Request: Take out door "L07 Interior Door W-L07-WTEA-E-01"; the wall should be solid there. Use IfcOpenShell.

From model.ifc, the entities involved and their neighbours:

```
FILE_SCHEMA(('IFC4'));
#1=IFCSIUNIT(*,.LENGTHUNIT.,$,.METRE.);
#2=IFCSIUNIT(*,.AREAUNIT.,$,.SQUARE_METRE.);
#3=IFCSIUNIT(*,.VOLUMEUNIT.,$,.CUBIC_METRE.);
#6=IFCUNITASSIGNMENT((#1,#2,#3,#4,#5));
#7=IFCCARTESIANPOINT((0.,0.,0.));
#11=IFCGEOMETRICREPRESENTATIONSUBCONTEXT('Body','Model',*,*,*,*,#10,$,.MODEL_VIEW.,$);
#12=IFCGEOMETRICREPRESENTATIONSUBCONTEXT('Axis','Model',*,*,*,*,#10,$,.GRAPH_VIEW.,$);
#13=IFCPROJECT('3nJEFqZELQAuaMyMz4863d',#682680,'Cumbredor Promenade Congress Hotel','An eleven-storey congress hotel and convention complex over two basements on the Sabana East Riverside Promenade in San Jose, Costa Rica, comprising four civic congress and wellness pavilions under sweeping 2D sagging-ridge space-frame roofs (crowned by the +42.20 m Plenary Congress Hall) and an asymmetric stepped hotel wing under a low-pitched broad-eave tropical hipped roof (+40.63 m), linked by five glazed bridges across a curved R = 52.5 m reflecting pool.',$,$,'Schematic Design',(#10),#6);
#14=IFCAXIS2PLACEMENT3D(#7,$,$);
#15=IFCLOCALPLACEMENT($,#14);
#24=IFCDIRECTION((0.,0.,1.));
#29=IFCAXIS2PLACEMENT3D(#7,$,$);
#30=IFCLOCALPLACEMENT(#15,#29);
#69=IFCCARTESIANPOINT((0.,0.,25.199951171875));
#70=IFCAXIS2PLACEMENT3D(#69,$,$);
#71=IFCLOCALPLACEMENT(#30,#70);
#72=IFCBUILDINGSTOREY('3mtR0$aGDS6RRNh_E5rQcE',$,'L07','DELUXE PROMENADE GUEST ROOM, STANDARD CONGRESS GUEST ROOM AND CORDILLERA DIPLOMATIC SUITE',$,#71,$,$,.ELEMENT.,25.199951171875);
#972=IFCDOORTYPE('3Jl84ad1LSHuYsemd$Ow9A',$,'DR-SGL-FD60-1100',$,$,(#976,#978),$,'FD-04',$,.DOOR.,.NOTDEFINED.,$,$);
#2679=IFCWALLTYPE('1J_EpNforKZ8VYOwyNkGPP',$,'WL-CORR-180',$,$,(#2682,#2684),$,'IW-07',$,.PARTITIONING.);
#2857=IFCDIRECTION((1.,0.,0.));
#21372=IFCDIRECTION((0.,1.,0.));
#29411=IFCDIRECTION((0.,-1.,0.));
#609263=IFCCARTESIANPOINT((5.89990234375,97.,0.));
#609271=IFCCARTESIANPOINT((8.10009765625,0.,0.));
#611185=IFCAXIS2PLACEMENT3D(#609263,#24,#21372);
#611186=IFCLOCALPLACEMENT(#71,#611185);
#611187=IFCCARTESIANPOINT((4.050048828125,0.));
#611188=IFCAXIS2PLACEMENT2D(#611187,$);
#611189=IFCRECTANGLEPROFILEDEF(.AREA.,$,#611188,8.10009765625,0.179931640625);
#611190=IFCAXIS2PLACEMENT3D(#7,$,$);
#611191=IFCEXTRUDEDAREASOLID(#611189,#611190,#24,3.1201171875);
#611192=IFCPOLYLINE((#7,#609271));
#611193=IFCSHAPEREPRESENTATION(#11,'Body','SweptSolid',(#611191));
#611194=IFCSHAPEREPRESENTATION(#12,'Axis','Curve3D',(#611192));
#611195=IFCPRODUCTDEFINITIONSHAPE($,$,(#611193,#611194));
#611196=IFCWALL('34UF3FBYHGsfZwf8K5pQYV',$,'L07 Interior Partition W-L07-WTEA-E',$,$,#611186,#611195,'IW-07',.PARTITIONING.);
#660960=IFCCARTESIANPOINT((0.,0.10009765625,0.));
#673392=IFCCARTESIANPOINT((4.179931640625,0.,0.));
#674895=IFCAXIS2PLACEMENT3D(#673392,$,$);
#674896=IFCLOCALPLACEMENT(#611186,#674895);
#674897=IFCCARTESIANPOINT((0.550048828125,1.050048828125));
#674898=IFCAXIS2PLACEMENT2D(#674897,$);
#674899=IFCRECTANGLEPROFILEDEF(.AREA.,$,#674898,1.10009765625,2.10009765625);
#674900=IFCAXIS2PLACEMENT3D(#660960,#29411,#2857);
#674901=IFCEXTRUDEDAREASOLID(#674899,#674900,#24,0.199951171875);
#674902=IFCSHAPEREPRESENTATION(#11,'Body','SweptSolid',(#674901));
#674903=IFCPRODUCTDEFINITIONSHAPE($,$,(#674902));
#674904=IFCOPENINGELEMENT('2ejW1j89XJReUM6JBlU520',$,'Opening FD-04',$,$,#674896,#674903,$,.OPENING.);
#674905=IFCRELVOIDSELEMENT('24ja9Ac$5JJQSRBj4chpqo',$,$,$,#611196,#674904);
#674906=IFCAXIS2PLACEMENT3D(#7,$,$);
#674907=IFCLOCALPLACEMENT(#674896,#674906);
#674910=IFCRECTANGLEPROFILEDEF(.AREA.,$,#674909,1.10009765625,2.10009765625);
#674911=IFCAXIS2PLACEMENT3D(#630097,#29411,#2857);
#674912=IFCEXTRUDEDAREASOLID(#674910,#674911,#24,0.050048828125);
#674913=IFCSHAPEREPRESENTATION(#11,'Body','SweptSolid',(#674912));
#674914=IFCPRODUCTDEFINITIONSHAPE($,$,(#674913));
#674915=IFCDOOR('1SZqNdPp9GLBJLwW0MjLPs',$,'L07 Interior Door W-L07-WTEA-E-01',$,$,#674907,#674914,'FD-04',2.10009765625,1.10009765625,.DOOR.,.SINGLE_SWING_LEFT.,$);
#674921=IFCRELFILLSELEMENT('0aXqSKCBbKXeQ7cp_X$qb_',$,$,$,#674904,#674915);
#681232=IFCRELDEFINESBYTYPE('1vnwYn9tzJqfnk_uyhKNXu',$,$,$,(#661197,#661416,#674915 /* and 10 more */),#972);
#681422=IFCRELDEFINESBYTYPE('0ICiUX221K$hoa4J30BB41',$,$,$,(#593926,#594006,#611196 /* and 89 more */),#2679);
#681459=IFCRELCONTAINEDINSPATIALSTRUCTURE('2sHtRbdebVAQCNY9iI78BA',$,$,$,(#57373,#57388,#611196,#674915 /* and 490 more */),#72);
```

```python
import ifcopenshell
import ifcopenshell.api.feature
import ifcopenshell.api.root
import ifcopenshell.geom
import ifcopenshell.util.shape

model = ifcopenshell.open("model.ifc")
settings = ifcopenshell.geom.settings()


def volume(element):
    """Net volume in cubic metres, openings subtracted."""
    shape = ifcopenshell.geom.create_shape(settings, element)
    return ifcopenshell.util.shape.get_volume(shape.geometry)


door = model.by_id(674915)
opening = door.FillsVoids[0].RelatingOpeningElement
wall = opening.VoidsElements[0].RelatingBuildingElement
before = volume(wall)

ifcopenshell.api.root.remove_product(model, product=door)
ifcopenshell.api.feature.remove_feature(model, feature=opening)

after = volume(wall)

print(f"wall volume {before:.3f} -> {after:.3f} m3")

model.write("model_updated.ifc")
```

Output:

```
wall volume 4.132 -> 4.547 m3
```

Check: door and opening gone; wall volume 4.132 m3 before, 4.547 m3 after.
